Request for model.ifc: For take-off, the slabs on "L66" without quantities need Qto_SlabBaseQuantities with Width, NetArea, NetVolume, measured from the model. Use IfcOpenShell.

First a look at what the model holds.

```python
import ifcopenshell
import ifcopenshell.util.element
import ifcopenshell.util.unit

model = ifcopenshell.open("model.ifc")
print(model.schema)
for unit_type in ("LENGTHUNIT", "AREAUNIT", "VOLUMEUNIT"):
    print(unit_type, ifcopenshell.util.unit.calculate_unit_scale(model, unit_type))
storey = next(s for s in model.by_type("IfcBuildingStorey") if s.Name == "L66")
slabs = [e for e in ifcopenshell.util.element.get_decomposition(storey) if e.is_a("IfcSlab")]
for e in sorted(slabs, key=lambda e: e.id()):
    print(e.id(), e.is_a(), e.Name, list(ifcopenshell.util.element.get_psets(e, qtos_only=True)), sep=" | ")
```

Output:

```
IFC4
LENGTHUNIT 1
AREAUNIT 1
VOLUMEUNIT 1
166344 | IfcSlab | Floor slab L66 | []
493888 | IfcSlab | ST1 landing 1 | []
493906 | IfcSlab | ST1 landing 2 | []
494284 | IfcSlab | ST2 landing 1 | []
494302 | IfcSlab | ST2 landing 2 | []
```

```python
import ifcopenshell
import ifcopenshell.api.pset
import ifcopenshell.geom
import ifcopenshell.util.element
import ifcopenshell.util.shape
import ifcopenshell.util.unit

model = ifcopenshell.open("model.ifc")
unit_scale = ifcopenshell.util.unit.calculate_unit_scale(model)
area_scale = ifcopenshell.util.unit.calculate_unit_scale(model, "AREAUNIT")
volume_scale = ifcopenshell.util.unit.calculate_unit_scale(model, "VOLUMEUNIT")
settings = ifcopenshell.geom.settings()

storey = next(s for s in model.by_type("IfcBuildingStorey") if s.Name == "L66")
slabs = [e for e in ifcopenshell.util.element.get_decomposition(storey) if e.is_a("IfcSlab")]

for e in sorted(slabs, key=lambda e: e.id()):
    if ifcopenshell.util.element.get_psets(e, qtos_only=True, should_inherit=False):
        continue
    # Geometry comes back in metres, in the element's own axes.
    shape = ifcopenshell.geom.create_shape(settings, e)
    values = {
        "Width": ifcopenshell.util.shape.get_z(shape.geometry) / unit_scale,
        "NetArea": ifcopenshell.util.shape.get_footprint_area(shape.geometry) / area_scale,
        "NetVolume": ifcopenshell.util.shape.get_volume(shape.geometry) / volume_scale,
    }
    qto = ifcopenshell.api.pset.add_qto(model, product=e, name="Qto_SlabBaseQuantities")
    ifcopenshell.api.pset.edit_qto(model, qto=qto, properties=values)
    print(e.id(), {k: round(v, 3) for k, v in values.items()})

model.write("model-out.ifc")
```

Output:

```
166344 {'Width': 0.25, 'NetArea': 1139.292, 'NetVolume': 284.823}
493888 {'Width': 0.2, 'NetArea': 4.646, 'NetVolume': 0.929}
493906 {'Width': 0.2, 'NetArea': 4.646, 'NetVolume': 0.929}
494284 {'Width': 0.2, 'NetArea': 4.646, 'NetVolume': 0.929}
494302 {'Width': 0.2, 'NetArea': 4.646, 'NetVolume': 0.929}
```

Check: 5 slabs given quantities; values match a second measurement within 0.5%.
